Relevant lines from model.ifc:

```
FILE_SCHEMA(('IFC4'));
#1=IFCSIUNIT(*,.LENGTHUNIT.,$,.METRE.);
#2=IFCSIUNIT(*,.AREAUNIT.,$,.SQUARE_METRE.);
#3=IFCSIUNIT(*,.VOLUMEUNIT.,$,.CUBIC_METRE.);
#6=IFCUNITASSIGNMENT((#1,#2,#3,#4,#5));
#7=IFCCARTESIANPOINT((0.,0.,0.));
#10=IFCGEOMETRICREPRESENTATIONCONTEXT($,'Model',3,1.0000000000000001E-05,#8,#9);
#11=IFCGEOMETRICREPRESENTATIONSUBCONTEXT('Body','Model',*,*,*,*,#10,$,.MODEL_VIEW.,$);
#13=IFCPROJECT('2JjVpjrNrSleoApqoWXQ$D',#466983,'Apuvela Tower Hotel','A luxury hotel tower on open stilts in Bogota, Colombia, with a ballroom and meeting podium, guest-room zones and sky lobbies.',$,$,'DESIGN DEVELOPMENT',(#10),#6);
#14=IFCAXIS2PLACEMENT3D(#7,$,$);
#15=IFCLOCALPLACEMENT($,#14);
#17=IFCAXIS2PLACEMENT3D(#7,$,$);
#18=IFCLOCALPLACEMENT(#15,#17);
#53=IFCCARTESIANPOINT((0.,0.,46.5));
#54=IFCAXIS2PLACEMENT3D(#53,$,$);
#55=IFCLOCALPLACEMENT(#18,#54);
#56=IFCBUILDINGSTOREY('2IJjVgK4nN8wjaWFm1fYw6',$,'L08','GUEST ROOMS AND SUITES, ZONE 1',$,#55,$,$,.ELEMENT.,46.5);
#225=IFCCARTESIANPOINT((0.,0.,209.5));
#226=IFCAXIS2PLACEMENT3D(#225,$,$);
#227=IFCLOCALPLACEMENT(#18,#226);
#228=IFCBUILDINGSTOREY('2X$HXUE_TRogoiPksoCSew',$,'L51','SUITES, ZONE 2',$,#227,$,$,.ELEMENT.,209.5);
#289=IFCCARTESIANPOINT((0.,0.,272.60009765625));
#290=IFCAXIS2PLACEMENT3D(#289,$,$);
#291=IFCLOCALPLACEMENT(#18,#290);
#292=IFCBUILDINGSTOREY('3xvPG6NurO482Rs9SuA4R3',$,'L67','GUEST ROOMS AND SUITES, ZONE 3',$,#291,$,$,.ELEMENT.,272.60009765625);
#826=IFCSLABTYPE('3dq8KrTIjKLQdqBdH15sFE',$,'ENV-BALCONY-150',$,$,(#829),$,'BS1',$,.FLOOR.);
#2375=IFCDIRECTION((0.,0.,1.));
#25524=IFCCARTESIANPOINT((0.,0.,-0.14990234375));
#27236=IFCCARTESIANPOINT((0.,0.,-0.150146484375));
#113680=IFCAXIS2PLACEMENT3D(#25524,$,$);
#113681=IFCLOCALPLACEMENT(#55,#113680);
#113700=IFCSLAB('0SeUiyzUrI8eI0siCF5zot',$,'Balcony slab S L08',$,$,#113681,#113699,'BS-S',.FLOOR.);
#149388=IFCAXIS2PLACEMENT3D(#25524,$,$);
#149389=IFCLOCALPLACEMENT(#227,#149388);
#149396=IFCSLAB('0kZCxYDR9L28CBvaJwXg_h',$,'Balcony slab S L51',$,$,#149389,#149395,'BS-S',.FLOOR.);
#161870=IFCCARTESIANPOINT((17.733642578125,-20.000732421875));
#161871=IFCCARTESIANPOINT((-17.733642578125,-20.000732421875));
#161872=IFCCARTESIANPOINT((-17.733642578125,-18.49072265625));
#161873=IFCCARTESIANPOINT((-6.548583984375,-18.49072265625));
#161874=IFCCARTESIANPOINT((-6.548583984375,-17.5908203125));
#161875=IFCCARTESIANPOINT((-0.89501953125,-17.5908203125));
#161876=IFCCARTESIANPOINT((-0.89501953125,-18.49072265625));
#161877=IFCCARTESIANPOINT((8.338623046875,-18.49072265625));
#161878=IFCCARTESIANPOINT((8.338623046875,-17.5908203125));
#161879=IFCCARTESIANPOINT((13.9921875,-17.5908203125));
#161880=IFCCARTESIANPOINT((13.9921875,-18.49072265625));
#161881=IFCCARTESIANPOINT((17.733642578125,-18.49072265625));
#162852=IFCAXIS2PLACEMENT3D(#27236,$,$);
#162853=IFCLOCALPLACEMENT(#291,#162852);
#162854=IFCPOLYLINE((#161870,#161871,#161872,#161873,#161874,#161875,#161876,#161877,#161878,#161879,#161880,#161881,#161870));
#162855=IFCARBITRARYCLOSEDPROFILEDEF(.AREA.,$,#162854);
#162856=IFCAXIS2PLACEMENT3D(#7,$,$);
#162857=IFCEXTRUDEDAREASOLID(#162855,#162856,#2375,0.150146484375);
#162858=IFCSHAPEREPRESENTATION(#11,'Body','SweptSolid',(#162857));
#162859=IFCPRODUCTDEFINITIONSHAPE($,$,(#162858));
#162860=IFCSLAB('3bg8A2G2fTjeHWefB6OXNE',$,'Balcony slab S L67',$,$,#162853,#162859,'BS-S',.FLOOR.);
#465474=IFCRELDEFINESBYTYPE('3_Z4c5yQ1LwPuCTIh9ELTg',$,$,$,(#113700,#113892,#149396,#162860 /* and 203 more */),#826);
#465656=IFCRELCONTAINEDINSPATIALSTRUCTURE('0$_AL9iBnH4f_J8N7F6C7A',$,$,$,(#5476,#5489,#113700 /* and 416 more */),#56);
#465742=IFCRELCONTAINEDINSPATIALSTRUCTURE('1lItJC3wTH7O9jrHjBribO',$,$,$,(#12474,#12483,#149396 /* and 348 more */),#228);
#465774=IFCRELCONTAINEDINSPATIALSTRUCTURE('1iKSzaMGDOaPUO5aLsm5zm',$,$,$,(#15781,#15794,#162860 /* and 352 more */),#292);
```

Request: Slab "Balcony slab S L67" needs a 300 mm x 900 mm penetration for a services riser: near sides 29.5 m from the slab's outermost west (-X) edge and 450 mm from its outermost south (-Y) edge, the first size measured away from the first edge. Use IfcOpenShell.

```python
import numpy as np
import ifcopenshell
import ifcopenshell.api.feature
import ifcopenshell.api.geometry
import ifcopenshell.api.root
import ifcopenshell.geom
import ifcopenshell.util.placement
import ifcopenshell.util.representation
import ifcopenshell.util.shape
import ifcopenshell.util.unit

model = ifcopenshell.open("model.ifc")
unit_scale = ifcopenshell.util.unit.calculate_unit_scale(model)
settings = ifcopenshell.geom.settings()


def volume(element):
    """Net volume in cubic metres, openings subtracted."""
    shape = ifcopenshell.geom.create_shape(settings, element)
    return ifcopenshell.util.shape.get_volume(shape.geometry)


slab = model.by_id(162860)
before = volume(slab)

# Extent in the slab's own axes, in metres. The edges named are its -X and -Y sides.
slab_shape = ifcopenshell.geom.create_shape(settings, slab)
vertices = ifcopenshell.util.shape.get_vertices(slab_shape.geometry)
x_min, y_min, bottom = vertices.min(axis=0)
top = vertices[:, 2].max()

opening = ifcopenshell.api.root.create_entity(model, ifc_class="IfcOpeningElement", name="Services riser opening", predefined_type="OPENING")
context = ifcopenshell.util.representation.get_context(model, "Model", "Body", "MODEL_VIEW")
width, depth = 0.3, 0.9
outline = [(0.0, 0.0), (width, 0.0), (width, depth), (0.0, depth), (0.0, 0.0)]
# Overshoot both faces by 50 mm so the cut is clean.
shape = ifcopenshell.api.geometry.add_slab_representation(
    model, context=context, depth=top - bottom + 0.1, polyline=outline
)
ifcopenshell.api.geometry.assign_representation(model, product=opening, representation=shape)

matrix = ifcopenshell.util.placement.get_local_placement(slab.ObjectPlacement)
matrix[:, 3] = matrix @ np.append(np.array([x_min + 29.5, y_min + 0.45, bottom - 0.05]) / unit_scale, 1.0)
ifcopenshell.api.geometry.edit_object_placement(model, product=opening, matrix=matrix, is_si=False)
ifcopenshell.api.feature.add_feature(model, feature=opening, element=slab)

after = volume(slab)

print(f"slab volume {before:.3f} -> {after:.3f} m3")

model.write("model_v2.ifc")
```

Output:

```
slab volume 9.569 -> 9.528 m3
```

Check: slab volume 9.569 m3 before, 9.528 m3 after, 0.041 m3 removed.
